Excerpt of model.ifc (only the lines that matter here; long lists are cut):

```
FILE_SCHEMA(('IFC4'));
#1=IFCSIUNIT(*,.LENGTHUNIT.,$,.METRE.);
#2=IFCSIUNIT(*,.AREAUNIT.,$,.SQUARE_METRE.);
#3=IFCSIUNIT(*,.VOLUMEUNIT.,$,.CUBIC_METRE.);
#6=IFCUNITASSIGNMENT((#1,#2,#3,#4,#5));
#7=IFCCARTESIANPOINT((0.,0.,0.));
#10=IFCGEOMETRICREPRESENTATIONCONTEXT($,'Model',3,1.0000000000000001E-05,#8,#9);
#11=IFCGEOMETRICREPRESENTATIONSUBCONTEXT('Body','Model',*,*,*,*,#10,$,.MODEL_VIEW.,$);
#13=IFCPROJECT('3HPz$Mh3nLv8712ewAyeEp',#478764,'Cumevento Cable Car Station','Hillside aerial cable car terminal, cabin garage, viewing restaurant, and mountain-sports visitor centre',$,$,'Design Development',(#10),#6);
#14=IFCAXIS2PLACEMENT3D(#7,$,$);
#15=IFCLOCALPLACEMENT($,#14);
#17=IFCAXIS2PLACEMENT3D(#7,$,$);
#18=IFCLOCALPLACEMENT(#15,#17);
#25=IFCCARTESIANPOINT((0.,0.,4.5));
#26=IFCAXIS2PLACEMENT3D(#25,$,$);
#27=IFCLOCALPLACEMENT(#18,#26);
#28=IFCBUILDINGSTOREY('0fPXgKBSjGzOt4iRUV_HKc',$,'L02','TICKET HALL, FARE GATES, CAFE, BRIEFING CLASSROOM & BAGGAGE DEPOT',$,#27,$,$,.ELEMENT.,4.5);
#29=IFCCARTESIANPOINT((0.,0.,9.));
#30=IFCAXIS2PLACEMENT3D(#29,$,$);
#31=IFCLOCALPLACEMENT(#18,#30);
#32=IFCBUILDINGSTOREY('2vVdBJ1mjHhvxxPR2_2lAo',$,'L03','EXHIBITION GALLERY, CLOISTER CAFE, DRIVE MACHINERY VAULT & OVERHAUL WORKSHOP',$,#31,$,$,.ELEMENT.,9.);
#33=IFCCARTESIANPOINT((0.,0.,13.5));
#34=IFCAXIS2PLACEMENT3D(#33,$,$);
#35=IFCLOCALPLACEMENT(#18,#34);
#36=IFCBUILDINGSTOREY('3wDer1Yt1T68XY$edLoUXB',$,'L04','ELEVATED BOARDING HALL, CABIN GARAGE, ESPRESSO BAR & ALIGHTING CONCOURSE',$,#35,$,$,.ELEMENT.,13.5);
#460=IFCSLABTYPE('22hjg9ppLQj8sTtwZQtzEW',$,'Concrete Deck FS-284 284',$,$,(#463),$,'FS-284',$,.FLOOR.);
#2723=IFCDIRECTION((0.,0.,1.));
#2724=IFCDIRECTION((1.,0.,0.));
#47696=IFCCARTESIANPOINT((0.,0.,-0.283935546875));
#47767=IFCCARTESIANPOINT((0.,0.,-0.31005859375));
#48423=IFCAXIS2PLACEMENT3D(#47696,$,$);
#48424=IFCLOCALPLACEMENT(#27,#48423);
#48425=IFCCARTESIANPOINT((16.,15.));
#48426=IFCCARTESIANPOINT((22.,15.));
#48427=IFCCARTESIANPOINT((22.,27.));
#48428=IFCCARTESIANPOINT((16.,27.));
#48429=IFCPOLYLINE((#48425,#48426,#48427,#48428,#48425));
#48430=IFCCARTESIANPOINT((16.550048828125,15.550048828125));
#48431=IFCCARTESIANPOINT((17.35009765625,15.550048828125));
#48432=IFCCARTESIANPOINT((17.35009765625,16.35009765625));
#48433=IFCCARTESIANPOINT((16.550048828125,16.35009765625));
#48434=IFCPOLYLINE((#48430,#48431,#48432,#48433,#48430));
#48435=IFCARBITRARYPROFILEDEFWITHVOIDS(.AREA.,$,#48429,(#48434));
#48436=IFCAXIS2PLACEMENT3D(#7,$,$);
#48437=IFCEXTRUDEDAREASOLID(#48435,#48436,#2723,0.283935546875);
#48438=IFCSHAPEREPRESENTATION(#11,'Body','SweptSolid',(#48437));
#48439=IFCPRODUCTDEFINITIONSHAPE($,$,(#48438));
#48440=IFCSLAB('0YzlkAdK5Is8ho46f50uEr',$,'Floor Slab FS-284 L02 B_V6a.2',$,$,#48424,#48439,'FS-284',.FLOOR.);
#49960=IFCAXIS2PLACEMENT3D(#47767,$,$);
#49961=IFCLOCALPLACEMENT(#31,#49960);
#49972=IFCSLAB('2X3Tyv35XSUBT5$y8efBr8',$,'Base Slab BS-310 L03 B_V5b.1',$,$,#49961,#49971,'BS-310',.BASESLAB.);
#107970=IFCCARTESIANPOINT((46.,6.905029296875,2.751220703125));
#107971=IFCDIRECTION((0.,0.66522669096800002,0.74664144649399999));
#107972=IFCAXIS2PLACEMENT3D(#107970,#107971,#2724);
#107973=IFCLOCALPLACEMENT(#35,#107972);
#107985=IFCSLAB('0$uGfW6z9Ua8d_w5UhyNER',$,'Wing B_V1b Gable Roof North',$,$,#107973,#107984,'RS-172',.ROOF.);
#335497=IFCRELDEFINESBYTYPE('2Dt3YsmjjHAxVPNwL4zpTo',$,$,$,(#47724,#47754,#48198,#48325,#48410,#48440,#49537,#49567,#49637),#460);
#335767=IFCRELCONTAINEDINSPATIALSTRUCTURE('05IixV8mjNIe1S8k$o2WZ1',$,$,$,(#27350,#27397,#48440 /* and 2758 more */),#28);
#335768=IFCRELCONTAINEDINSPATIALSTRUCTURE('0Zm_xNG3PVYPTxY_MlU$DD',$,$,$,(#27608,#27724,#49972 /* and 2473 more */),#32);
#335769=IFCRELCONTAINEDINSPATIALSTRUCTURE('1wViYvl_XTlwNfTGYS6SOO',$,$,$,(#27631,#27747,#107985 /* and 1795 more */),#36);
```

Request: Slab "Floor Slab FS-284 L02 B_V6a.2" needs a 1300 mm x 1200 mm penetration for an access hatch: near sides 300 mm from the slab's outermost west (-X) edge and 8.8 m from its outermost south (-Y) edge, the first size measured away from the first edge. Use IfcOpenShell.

```python
import numpy as np
import ifcopenshell
import ifcopenshell.api.feature
import ifcopenshell.api.geometry
import ifcopenshell.api.root
import ifcopenshell.geom
import ifcopenshell.util.placement
import ifcopenshell.util.representation
import ifcopenshell.util.shape
import ifcopenshell.util.unit

model = ifcopenshell.open("model.ifc")
unit_scale = ifcopenshell.util.unit.calculate_unit_scale(model)
settings = ifcopenshell.geom.settings()


def volume(element):
    """Net volume in cubic metres, openings subtracted."""
    shape = ifcopenshell.geom.create_shape(settings, element)
    return ifcopenshell.util.shape.get_volume(shape.geometry)


slab = model.by_guid("0YzlkAdK5Is8ho46f50uEr")
before = volume(slab)

# Extent in the slab's own axes, in metres. The edges named are its -X and -Y sides.
slab_shape = ifcopenshell.geom.create_shape(settings, slab)
vertices = ifcopenshell.util.shape.get_vertices(slab_shape.geometry)
x_min, y_min, bottom = vertices.min(axis=0)
top = vertices[:, 2].max()

opening = ifcopenshell.api.root.create_entity(model, ifc_class="IfcOpeningElement", name="Access hatch opening", predefined_type="OPENING")
context = ifcopenshell.util.representation.get_context(model, "Model", "Body", "MODEL_VIEW")
width, depth = 1.3, 1.2
outline = [(0.0, 0.0), (width, 0.0), (width, depth), (0.0, depth), (0.0, 0.0)]
# Overshoot both faces by 50 mm so the cut is clean.
shape = ifcopenshell.api.geometry.add_slab_representation(
    model, context=context, depth=top - bottom + 0.1, polyline=outline
)
ifcopenshell.api.geometry.assign_representation(model, product=opening, representation=shape)

matrix = ifcopenshell.util.placement.get_local_placement(slab.ObjectPlacement)
matrix[:, 3] = matrix @ np.append(np.array([x_min + 0.3, y_min + 8.8, bottom - 0.05]) / unit_scale, 1.0)
ifcopenshell.api.geometry.edit_object_placement(model, product=opening, matrix=matrix, is_si=False)
ifcopenshell.api.feature.add_feature(model, feature=opening, element=slab)

after = volume(slab)

print(f"slab volume {before:.3f} -> {after:.3f} m3")

model.write("model_rev.ifc")
```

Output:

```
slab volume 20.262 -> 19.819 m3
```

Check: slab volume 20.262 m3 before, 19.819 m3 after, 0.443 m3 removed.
